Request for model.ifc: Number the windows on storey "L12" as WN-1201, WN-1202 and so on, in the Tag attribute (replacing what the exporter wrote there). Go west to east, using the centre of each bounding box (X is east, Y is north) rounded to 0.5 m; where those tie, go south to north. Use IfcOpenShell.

First a look at what the model holds.

```python
import ifcopenshell
import ifcopenshell.util.element
import ifcopenshell.util.placement

model = ifcopenshell.open("model.ifc")
print(model.schema)
storey = next(s for s in model.by_type("IfcBuildingStorey") if s.Name == "L12")
windows = [e for e in ifcopenshell.util.element.get_decomposition(storey) if e.is_a("IfcWindow")]
for e in sorted(windows, key=lambda e: e.id()):
    origin = ifcopenshell.util.placement.get_local_placement(e.ObjectPlacement)[:3, 3]
    print(e.id(), e.Tag, e.Name, origin.round(2) + 0.0, sep=" | ")
```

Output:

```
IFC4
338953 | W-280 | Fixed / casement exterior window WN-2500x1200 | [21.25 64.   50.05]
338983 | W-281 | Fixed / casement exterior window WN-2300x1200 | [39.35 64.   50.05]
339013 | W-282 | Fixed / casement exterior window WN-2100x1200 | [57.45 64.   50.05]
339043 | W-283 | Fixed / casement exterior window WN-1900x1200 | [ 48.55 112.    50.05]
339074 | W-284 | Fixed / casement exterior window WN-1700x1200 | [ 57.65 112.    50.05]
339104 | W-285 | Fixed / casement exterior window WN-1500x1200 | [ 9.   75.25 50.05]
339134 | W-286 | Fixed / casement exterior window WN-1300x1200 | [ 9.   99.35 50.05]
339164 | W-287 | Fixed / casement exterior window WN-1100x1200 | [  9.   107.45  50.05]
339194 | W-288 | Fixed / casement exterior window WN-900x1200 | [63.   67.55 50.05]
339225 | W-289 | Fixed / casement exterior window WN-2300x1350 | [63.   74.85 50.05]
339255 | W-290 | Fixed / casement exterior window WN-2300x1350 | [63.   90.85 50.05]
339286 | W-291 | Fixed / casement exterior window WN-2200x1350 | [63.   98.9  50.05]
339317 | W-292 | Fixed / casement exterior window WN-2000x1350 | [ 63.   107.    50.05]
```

```python
import ifcopenshell
import ifcopenshell.geom
import ifcopenshell.util.element
import ifcopenshell.util.shape

model = ifcopenshell.open("model.ifc")
settings = ifcopenshell.geom.settings()
settings.set("use-world-coords", True)


def centre(element):
    shape = ifcopenshell.geom.create_shape(settings, element)
    return ifcopenshell.util.shape.get_bbox_centroid(shape.geometry)


storey = next(s for s in model.by_type("IfcBuildingStorey") if s.Name == "L12")
windows = [e for e in ifcopenshell.util.element.get_decomposition(storey) if e.is_a("IfcWindow")]

# Insertion points can sit at a corner or the storey origin, so sort by the geometry (in metres).
centres = {e: centre(e) for e in windows}
windows.sort(key=lambda e: (round(centres[e][0] / 0.5), centres[e][1]))

for i, e in enumerate(windows, start=1):
    number = f"WN-12{i:02d}"
    e.Tag = number
    print(e.id(), number)

model.write("model_updated.ifc")
```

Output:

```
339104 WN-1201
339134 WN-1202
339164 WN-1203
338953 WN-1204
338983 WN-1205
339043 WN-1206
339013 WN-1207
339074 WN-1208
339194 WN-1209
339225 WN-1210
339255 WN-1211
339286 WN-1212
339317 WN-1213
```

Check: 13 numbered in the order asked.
